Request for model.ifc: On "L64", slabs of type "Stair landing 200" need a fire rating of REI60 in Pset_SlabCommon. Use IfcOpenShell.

First a look at what the model holds.

```python
import ifcopenshell
import ifcopenshell.util.element

model = ifcopenshell.open("model.ifc")
print(model.schema)
storey = next(s for s in model.by_type("IfcBuildingStorey") if s.Name == "L64")
slabs = [e for e in ifcopenshell.util.element.get_decomposition(storey) if e.is_a("IfcSlab")]
seen = {}
for e in slabs:
    element_type = ifcopenshell.util.element.get_type(e)
    key = (element_type.Name if element_type != e and element_type else None, ifcopenshell.util.element.get_pset(e, "Pset_SlabCommon", "FireRating"))
    seen[key] = seen.get(key, 0) + 1
for (name, value), count in sorted(seen.items(), key=str):
    print(count, "x", name, "|", value)
```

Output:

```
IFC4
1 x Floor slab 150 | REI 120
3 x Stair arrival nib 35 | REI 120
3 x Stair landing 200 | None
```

```python
import ifcopenshell
import ifcopenshell.api.pset
import ifcopenshell.util.element

model = ifcopenshell.open("model.ifc")

storey = next(s for s in model.by_type("IfcBuildingStorey") if s.Name == "L64")
slabs = [e for e in ifcopenshell.util.element.get_decomposition(storey) if e.is_a("IfcSlab")]

count = 0
for e in slabs:
    element_type = ifcopenshell.util.element.get_type(e)
    if element_type in (None, e) or element_type.Name != "Stair landing 200":
        continue
    found = ifcopenshell.util.element.get_pset(e, "Pset_SlabCommon", should_inherit=False)
    if found:
        pset = model.by_id(found["id"])
        if len(ifcopenshell.util.element.get_elements_by_pset(pset)) > 1:
            pset = ifcopenshell.api.pset.unshare_pset(model, products=[e], pset=pset)[0]
    else:
        pset = ifcopenshell.api.pset.add_pset(model, product=e, name="Pset_SlabCommon")
    ifcopenshell.api.pset.edit_pset(model, pset=pset, properties={"FireRating": "REI60"})
    count += 1

print(count, "slabs updated")

model.write("model_v2.ifc")
```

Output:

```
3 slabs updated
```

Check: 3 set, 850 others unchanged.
